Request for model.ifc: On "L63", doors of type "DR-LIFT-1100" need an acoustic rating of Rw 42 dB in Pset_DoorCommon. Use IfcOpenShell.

First a look at what the model holds.

```python
import ifcopenshell
import ifcopenshell.util.element

model = ifcopenshell.open("model.ifc")
print(model.schema)
storey = next(s for s in model.by_type("IfcBuildingStorey") if s.Name == "L63")
doors = [e for e in ifcopenshell.util.element.get_decomposition(storey) if e.is_a("IfcDoor")]
seen = {}
for e in doors:
    element_type = ifcopenshell.util.element.get_type(e)
    key = (element_type.Name if element_type != e and element_type else None, ifcopenshell.util.element.get_pset(e, "Pset_DoorCommon", "AcousticRating"))
    seen[key] = seen.get(key, 0) + 1
for (name, value), count in sorted(seen.items(), key=str):
    print(count, "x", name, "|", value)
```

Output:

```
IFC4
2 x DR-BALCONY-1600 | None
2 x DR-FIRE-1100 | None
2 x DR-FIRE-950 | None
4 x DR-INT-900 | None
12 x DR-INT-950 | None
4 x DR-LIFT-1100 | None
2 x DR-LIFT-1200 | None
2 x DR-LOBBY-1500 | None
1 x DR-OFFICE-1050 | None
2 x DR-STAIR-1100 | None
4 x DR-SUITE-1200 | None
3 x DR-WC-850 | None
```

```python
import ifcopenshell
import ifcopenshell.api.pset
import ifcopenshell.util.element

model = ifcopenshell.open("model.ifc")

storey = next(s for s in model.by_type("IfcBuildingStorey") if s.Name == "L63")
doors = [e for e in ifcopenshell.util.element.get_decomposition(storey) if e.is_a("IfcDoor")]

count = 0
for e in doors:
    element_type = ifcopenshell.util.element.get_type(e)
    if element_type in (None, e) or element_type.Name != "DR-LIFT-1100":
        continue
    found = ifcopenshell.util.element.get_pset(e, "Pset_DoorCommon", should_inherit=False)
    if found:
        pset = model.by_id(found["id"])
        if len(ifcopenshell.util.element.get_elements_by_pset(pset)) > 1:
            pset = ifcopenshell.api.pset.unshare_pset(model, products=[e], pset=pset)[0]
    else:
        pset = ifcopenshell.api.pset.add_pset(model, product=e, name="Pset_DoorCommon")
    ifcopenshell.api.pset.edit_pset(model, pset=pset, properties={"AcousticRating": "Rw 42 dB"})
    count += 1

print(count, "doors updated")

model.write("model_updated.ifc")
```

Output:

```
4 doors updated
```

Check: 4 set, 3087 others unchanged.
